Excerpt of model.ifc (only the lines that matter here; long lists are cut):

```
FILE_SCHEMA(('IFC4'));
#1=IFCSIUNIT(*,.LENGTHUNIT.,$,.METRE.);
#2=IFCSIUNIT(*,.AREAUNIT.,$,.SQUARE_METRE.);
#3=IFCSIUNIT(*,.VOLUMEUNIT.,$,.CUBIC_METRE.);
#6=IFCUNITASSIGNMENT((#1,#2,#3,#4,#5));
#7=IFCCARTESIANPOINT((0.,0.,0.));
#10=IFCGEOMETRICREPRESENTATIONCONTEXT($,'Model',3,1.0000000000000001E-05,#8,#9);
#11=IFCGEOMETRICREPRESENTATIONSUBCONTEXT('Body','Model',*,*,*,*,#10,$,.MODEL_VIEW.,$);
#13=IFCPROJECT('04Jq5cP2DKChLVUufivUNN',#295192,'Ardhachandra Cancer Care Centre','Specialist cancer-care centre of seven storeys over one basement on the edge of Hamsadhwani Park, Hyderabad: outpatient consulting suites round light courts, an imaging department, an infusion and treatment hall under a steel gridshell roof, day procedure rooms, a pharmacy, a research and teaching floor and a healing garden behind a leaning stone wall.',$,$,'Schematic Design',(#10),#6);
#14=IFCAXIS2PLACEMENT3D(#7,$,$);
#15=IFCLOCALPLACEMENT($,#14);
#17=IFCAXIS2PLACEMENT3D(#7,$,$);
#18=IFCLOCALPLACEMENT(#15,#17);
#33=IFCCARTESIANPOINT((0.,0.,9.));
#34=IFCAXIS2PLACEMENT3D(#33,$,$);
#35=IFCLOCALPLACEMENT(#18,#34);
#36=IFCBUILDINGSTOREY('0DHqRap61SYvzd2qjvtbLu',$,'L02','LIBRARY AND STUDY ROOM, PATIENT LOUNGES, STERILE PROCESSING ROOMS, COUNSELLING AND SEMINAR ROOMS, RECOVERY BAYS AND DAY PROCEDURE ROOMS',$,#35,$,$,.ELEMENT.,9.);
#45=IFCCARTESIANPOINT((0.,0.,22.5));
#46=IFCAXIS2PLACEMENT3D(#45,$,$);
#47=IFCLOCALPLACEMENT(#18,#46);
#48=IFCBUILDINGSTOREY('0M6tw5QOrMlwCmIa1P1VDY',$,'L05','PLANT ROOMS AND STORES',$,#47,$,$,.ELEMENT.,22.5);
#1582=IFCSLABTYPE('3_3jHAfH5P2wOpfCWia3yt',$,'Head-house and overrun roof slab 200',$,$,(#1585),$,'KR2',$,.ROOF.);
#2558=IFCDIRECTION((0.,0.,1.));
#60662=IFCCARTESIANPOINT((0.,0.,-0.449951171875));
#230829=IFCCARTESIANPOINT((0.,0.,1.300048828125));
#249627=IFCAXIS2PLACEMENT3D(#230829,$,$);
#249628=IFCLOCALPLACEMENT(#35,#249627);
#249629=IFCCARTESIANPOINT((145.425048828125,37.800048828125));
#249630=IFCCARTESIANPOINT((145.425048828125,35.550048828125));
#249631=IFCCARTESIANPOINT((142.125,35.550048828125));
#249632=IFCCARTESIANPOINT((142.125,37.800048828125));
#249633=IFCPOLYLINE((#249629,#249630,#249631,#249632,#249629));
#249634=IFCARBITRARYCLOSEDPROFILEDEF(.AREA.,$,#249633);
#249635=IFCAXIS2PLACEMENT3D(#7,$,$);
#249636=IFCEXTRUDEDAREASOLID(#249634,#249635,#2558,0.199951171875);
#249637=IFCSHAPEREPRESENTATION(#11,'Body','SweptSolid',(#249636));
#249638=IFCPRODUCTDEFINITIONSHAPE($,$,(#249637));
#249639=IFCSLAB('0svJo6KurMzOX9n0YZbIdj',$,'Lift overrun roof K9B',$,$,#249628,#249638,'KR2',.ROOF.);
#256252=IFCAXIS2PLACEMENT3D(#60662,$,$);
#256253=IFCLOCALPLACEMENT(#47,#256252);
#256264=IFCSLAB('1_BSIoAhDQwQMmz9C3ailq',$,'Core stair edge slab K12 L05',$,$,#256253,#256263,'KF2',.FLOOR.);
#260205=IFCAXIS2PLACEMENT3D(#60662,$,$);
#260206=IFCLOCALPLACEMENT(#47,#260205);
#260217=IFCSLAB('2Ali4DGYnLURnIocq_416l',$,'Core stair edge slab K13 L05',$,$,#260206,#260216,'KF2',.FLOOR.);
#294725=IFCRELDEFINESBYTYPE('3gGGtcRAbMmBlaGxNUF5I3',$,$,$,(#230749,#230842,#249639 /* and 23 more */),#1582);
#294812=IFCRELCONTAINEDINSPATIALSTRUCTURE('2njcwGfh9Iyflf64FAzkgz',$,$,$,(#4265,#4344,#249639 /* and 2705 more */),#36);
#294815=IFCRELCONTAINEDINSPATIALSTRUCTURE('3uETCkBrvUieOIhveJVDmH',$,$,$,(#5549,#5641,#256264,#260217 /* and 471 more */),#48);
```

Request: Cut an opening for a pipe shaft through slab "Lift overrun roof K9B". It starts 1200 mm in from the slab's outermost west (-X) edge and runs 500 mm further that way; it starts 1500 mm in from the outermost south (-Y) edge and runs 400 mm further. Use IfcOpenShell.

```python
import numpy as np
import ifcopenshell
import ifcopenshell.api.feature
import ifcopenshell.api.geometry
import ifcopenshell.api.root
import ifcopenshell.geom
import ifcopenshell.util.placement
import ifcopenshell.util.representation
import ifcopenshell.util.shape
import ifcopenshell.util.unit

model = ifcopenshell.open("model.ifc")
unit_scale = ifcopenshell.util.unit.calculate_unit_scale(model)
settings = ifcopenshell.geom.settings()


def volume(element):
    """Net volume in cubic metres, openings subtracted."""
    shape = ifcopenshell.geom.create_shape(settings, element)
    return ifcopenshell.util.shape.get_volume(shape.geometry)


slab = model.by_guid("0svJo6KurMzOX9n0YZbIdj")
before = volume(slab)

# Extent in the slab's own axes, in metres. The edges named are its -X and -Y sides.
slab_shape = ifcopenshell.geom.create_shape(settings, slab)
vertices = ifcopenshell.util.shape.get_vertices(slab_shape.geometry)
x_min, y_min, bottom = vertices.min(axis=0)
top = vertices[:, 2].max()

opening = ifcopenshell.api.root.create_entity(model, ifc_class="IfcOpeningElement", name="Pipe shaft opening", predefined_type="OPENING")
context = ifcopenshell.util.representation.get_context(model, "Model", "Body", "MODEL_VIEW")
width, depth = 0.5, 0.4
outline = [(0.0, 0.0), (width, 0.0), (width, depth), (0.0, depth), (0.0, 0.0)]
# Overshoot both faces by 50 mm so the cut is clean.
shape = ifcopenshell.api.geometry.add_slab_representation(
    model, context=context, depth=top - bottom + 0.1, polyline=outline
)
ifcopenshell.api.geometry.assign_representation(model, product=opening, representation=shape)

matrix = ifcopenshell.util.placement.get_local_placement(slab.ObjectPlacement)
matrix[:, 3] = matrix @ np.append(np.array([x_min + 1.2, y_min + 1.5, bottom - 0.05]) / unit_scale, 1.0)
ifcopenshell.api.geometry.edit_object_placement(model, product=opening, matrix=matrix, is_si=False)
ifcopenshell.api.feature.add_feature(model, feature=opening, element=slab)

after = volume(slab)

print(f"slab volume {before:.3f} -> {after:.3f} m3")

model.write("model_rev.ifc")
```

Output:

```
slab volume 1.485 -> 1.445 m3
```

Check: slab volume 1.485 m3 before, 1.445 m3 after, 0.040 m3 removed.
